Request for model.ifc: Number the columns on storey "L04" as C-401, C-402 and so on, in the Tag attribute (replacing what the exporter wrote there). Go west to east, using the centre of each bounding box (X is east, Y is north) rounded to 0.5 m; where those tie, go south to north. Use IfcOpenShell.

First a look at what the model holds.

```python
import ifcopenshell
import ifcopenshell.util.element
import ifcopenshell.util.placement

model = ifcopenshell.open("model.ifc")
print(model.schema)
storey = next(s for s in model.by_type("IfcBuildingStorey") if s.Name == "L04")
columns = [e for e in ifcopenshell.util.element.get_decomposition(storey) if e.is_a("IfcColumn")]
for e in sorted(columns, key=lambda e: e.id()):
    origin = ifcopenshell.util.placement.get_local_placement(e.ObjectPlacement)[:3, 3]
    print(e.id(), e.Tag, e.Name, origin.round(2) + 0.0, sep=" | ")
```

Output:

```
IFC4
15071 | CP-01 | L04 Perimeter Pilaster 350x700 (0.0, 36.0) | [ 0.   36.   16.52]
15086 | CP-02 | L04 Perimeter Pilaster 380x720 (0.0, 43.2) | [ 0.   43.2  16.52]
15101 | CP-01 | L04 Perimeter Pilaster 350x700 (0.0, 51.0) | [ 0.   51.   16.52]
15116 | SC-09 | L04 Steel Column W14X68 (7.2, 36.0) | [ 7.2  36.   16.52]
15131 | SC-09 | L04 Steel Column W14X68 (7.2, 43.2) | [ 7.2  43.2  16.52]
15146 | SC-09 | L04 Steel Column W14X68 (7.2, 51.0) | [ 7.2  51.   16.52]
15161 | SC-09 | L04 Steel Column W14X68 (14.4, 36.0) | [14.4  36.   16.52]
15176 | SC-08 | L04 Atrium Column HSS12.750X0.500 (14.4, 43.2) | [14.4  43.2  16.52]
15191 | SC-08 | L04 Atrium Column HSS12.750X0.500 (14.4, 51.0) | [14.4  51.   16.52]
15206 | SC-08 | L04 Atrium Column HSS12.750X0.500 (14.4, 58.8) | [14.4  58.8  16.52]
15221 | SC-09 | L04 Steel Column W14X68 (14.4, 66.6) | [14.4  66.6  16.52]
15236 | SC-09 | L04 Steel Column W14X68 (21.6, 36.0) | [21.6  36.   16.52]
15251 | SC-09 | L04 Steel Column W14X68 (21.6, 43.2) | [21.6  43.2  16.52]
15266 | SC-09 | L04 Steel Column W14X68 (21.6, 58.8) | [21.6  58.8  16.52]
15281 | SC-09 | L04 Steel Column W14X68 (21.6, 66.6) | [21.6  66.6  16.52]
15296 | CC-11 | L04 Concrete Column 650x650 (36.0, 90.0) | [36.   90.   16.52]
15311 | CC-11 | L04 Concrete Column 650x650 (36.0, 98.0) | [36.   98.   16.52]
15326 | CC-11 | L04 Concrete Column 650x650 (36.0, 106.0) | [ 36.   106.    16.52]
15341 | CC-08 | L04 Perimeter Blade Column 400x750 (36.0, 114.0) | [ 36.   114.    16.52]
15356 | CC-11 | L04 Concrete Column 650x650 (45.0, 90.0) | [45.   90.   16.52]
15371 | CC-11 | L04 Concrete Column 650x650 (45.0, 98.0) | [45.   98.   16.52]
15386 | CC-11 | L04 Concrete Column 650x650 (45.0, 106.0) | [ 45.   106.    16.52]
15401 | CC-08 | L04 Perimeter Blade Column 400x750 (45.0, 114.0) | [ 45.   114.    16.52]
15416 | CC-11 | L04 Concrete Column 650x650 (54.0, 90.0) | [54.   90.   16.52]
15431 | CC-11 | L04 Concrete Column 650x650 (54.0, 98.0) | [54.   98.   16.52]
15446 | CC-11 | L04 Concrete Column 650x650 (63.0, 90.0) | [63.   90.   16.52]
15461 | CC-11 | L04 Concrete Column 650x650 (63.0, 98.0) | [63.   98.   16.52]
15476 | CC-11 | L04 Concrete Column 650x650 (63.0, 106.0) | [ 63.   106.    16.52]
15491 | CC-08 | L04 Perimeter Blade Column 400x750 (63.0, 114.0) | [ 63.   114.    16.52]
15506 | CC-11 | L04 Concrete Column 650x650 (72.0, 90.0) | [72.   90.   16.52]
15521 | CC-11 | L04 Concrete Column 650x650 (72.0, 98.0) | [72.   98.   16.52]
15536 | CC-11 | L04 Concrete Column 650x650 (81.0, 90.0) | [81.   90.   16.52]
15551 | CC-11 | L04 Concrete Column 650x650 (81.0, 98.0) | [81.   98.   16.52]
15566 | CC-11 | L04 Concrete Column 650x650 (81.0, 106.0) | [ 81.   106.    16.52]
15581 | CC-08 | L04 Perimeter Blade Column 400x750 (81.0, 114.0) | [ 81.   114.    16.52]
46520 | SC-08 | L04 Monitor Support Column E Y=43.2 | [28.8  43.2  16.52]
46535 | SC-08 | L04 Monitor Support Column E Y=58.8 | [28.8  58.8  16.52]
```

```python
import ifcopenshell
import ifcopenshell.geom
import ifcopenshell.util.element
import ifcopenshell.util.shape

model = ifcopenshell.open("model.ifc")
settings = ifcopenshell.geom.settings()
settings.set("use-world-coords", True)


def centre(element):
    shape = ifcopenshell.geom.create_shape(settings, element)
    return ifcopenshell.util.shape.get_bbox_centroid(shape.geometry)


storey = next(s for s in model.by_type("IfcBuildingStorey") if s.Name == "L04")
columns = [e for e in ifcopenshell.util.element.get_decomposition(storey) if e.is_a("IfcColumn")]

# Insertion points can sit at a corner or the storey origin, so sort by the geometry (in metres).
centres = {e: centre(e) for e in columns}
columns.sort(key=lambda e: (round(centres[e][0] / 0.5), centres[e][1]))

for i, e in enumerate(columns, start=1):
    number = f"C-4{i:02d}"
    e.Tag = number
    print(e.id(), number)

model.write("model_edited.ifc")
```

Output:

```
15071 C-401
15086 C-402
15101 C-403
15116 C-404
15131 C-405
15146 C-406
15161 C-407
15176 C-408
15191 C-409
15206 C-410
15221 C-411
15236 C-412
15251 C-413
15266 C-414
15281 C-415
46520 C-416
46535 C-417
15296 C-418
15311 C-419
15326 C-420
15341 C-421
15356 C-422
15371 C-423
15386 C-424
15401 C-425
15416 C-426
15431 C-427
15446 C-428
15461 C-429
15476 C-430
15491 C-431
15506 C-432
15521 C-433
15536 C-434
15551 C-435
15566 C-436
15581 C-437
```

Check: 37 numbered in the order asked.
